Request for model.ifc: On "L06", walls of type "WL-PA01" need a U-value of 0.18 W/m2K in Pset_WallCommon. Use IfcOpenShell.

First a look at what the model holds.

```python
import ifcopenshell
import ifcopenshell.util.element

model = ifcopenshell.open("model.ifc")
print(model.schema)
storey = next(s for s in model.by_type("IfcBuildingStorey") if s.Name == "L06")
walls = [e for e in ifcopenshell.util.element.get_decomposition(storey) if e.is_a("IfcWall")]
seen = {}
for e in walls:
    element_type = ifcopenshell.util.element.get_type(e)
    key = (element_type.Name if element_type != e and element_type else None, ifcopenshell.util.element.get_pset(e, "Pset_WallCommon", "ThermalTransmittance"))
    seen[key] = seen.get(key, 0) + 1
for (name, value), count in sorted(seen.items(), key=str):
    print(count, "x", name, "|", value)
```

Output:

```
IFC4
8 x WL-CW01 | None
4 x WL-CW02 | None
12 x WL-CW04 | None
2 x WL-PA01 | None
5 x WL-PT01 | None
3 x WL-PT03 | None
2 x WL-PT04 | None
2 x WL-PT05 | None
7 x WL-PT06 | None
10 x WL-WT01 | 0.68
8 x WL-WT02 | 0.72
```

```python
import ifcopenshell
import ifcopenshell.api.pset
import ifcopenshell.util.element

model = ifcopenshell.open("model.ifc")

storey = next(s for s in model.by_type("IfcBuildingStorey") if s.Name == "L06")
walls = [e for e in ifcopenshell.util.element.get_decomposition(storey) if e.is_a("IfcWall")]

count = 0
for e in walls:
    element_type = ifcopenshell.util.element.get_type(e)
    if element_type in (None, e) or element_type.Name != "WL-PA01":
        continue
    # add_pset returns the element's existing set when there is one.
    pset = ifcopenshell.api.pset.add_pset(model, product=e, name="Pset_WallCommon")
    ifcopenshell.api.pset.edit_pset(model, pset=pset, properties={"ThermalTransmittance": 0.18})
    count += 1

print(count, "walls updated")

model.write("model-out.ifc")
```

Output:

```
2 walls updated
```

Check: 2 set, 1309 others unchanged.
